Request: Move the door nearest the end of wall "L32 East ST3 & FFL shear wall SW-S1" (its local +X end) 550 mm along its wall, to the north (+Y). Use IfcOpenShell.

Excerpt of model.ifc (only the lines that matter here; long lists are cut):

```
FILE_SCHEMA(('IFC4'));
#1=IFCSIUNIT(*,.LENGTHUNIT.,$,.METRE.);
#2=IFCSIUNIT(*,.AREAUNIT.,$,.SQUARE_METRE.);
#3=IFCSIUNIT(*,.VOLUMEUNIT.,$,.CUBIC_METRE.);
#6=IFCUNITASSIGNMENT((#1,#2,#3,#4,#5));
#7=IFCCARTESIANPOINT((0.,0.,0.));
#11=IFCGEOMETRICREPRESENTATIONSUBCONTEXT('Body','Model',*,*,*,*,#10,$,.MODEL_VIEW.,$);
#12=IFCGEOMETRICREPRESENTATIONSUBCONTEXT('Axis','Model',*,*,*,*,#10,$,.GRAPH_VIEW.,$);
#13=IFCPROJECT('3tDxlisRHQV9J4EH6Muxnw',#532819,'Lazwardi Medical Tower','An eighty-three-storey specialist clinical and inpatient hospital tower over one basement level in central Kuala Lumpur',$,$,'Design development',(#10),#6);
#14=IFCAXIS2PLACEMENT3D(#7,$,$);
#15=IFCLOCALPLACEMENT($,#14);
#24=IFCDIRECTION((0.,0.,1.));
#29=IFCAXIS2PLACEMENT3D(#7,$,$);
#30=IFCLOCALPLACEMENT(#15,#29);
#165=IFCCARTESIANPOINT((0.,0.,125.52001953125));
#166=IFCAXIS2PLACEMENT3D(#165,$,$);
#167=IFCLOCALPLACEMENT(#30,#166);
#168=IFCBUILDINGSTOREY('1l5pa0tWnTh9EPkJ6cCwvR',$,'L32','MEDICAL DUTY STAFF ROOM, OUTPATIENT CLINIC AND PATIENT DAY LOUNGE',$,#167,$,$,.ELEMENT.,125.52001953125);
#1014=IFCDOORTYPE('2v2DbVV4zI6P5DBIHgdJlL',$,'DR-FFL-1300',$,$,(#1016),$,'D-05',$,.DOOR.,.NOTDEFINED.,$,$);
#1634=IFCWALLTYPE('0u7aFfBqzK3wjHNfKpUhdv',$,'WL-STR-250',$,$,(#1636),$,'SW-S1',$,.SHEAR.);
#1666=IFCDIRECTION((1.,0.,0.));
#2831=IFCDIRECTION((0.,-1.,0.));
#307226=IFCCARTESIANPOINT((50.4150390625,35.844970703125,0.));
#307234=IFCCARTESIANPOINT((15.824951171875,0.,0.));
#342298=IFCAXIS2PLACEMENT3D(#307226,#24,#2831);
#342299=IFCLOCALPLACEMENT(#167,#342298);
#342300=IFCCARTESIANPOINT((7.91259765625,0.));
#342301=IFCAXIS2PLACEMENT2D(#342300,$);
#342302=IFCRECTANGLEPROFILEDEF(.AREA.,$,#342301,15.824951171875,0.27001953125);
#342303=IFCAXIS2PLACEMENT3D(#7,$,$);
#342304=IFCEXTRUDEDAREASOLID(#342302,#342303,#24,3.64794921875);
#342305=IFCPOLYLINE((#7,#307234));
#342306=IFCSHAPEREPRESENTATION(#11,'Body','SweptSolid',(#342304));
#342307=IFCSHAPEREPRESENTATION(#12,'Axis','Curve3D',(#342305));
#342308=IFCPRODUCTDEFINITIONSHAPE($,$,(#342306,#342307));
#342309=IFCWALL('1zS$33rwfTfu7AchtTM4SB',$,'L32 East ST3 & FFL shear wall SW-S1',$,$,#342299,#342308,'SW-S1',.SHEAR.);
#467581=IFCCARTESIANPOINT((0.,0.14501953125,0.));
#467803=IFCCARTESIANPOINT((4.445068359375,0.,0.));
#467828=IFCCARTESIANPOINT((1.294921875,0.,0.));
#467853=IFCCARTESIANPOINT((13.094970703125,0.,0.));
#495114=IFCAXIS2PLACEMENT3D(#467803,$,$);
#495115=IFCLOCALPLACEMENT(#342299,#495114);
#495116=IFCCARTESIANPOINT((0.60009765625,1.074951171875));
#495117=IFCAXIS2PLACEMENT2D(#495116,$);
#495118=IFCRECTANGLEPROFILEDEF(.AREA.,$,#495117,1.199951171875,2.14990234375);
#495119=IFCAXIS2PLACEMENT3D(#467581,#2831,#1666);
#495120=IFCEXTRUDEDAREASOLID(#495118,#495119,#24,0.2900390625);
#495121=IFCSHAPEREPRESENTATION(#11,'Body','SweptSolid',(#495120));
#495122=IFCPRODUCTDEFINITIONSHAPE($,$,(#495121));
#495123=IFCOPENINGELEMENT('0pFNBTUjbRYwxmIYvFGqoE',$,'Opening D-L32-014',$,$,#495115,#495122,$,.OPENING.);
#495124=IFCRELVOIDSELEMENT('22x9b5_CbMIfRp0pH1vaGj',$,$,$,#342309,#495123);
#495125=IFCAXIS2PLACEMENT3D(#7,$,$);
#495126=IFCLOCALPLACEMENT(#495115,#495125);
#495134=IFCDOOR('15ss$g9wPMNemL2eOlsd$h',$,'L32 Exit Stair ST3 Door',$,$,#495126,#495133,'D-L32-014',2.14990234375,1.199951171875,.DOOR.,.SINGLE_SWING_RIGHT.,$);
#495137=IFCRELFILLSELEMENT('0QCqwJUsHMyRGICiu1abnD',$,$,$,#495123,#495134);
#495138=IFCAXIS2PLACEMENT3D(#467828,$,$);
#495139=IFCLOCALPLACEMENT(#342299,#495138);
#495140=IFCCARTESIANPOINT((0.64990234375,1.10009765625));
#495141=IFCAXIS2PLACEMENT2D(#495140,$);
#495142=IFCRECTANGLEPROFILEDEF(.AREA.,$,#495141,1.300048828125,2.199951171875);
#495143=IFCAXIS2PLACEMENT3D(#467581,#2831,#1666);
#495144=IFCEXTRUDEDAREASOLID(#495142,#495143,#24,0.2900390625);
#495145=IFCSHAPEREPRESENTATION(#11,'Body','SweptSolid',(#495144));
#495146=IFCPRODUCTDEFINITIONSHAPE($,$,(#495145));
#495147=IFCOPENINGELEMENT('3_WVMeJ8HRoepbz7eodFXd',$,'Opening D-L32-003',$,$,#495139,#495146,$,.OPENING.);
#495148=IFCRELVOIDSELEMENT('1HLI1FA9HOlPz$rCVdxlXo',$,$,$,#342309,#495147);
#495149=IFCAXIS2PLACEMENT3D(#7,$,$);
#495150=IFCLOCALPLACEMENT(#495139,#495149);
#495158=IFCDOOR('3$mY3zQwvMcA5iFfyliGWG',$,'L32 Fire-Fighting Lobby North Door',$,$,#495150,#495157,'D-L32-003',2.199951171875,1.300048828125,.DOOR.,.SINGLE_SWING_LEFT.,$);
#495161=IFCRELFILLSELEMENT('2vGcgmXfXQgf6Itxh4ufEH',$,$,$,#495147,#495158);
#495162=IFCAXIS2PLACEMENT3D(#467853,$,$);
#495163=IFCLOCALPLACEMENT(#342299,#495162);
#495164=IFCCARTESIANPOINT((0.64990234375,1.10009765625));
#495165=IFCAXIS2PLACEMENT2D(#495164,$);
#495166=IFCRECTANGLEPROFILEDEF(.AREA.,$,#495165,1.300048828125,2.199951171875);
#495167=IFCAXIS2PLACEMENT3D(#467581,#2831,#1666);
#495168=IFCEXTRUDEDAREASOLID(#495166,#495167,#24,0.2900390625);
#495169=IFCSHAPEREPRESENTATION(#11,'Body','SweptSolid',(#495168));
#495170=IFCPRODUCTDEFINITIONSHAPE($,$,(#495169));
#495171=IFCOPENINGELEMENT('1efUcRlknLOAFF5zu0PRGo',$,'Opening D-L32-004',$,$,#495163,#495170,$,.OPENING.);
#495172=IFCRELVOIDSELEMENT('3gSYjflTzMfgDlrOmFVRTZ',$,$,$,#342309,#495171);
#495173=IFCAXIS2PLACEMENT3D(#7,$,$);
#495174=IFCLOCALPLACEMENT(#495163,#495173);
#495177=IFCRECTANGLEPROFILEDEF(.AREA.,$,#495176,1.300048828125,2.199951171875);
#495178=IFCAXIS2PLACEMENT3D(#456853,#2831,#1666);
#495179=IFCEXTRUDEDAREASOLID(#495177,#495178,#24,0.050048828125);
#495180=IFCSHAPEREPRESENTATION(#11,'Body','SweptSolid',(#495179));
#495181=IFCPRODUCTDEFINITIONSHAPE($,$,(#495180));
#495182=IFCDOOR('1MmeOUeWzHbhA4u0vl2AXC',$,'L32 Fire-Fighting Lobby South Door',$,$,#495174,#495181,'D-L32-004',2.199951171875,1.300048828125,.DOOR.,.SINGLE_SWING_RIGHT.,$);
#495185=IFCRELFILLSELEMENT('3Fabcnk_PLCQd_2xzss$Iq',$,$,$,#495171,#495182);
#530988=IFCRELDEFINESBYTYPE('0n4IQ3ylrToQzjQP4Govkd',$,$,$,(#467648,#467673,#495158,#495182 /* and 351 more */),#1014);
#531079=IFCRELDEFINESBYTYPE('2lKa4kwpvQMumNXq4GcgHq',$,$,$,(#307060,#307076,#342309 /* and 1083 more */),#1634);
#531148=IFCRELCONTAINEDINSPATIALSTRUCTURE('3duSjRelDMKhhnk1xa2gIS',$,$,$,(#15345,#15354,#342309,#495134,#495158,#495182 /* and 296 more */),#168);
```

```python
import ifcopenshell
import ifcopenshell.api.geometry
import ifcopenshell.util.placement
import ifcopenshell.util.unit

model = ifcopenshell.open("model.ifc")
unit_scale = ifcopenshell.util.unit.calculate_unit_scale(model)

door = model.by_guid("1MmeOUeWzHbhA4u0vl2AXC")
opening = door.FillsVoids[0].RelatingOpeningElement
wall = opening.VoidsElements[0].RelatingBuildingElement

wall_matrix = ifcopenshell.util.placement.get_local_placement(wall.ObjectPlacement)
shift = wall_matrix[:3, 0] * -0.55 / unit_scale
before = ifcopenshell.util.placement.get_local_placement(door.ObjectPlacement)[:3, 3].copy()

# The door is placed relative to its opening, so it follows when the opening moves.
matrix = ifcopenshell.util.placement.get_local_placement(opening.ObjectPlacement)
matrix[:3, 3] += shift
ifcopenshell.api.geometry.edit_object_placement(
    model, product=opening, matrix=matrix, is_si=False, should_transform_children=True
)

after = ifcopenshell.util.placement.get_local_placement(door.ObjectPlacement)[:3, 3]
print("door moved by", (after - before).round(3) + 0.0)

model.write("model_edited.ifc")
```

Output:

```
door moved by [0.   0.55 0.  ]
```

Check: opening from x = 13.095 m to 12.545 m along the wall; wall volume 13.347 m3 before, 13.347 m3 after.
